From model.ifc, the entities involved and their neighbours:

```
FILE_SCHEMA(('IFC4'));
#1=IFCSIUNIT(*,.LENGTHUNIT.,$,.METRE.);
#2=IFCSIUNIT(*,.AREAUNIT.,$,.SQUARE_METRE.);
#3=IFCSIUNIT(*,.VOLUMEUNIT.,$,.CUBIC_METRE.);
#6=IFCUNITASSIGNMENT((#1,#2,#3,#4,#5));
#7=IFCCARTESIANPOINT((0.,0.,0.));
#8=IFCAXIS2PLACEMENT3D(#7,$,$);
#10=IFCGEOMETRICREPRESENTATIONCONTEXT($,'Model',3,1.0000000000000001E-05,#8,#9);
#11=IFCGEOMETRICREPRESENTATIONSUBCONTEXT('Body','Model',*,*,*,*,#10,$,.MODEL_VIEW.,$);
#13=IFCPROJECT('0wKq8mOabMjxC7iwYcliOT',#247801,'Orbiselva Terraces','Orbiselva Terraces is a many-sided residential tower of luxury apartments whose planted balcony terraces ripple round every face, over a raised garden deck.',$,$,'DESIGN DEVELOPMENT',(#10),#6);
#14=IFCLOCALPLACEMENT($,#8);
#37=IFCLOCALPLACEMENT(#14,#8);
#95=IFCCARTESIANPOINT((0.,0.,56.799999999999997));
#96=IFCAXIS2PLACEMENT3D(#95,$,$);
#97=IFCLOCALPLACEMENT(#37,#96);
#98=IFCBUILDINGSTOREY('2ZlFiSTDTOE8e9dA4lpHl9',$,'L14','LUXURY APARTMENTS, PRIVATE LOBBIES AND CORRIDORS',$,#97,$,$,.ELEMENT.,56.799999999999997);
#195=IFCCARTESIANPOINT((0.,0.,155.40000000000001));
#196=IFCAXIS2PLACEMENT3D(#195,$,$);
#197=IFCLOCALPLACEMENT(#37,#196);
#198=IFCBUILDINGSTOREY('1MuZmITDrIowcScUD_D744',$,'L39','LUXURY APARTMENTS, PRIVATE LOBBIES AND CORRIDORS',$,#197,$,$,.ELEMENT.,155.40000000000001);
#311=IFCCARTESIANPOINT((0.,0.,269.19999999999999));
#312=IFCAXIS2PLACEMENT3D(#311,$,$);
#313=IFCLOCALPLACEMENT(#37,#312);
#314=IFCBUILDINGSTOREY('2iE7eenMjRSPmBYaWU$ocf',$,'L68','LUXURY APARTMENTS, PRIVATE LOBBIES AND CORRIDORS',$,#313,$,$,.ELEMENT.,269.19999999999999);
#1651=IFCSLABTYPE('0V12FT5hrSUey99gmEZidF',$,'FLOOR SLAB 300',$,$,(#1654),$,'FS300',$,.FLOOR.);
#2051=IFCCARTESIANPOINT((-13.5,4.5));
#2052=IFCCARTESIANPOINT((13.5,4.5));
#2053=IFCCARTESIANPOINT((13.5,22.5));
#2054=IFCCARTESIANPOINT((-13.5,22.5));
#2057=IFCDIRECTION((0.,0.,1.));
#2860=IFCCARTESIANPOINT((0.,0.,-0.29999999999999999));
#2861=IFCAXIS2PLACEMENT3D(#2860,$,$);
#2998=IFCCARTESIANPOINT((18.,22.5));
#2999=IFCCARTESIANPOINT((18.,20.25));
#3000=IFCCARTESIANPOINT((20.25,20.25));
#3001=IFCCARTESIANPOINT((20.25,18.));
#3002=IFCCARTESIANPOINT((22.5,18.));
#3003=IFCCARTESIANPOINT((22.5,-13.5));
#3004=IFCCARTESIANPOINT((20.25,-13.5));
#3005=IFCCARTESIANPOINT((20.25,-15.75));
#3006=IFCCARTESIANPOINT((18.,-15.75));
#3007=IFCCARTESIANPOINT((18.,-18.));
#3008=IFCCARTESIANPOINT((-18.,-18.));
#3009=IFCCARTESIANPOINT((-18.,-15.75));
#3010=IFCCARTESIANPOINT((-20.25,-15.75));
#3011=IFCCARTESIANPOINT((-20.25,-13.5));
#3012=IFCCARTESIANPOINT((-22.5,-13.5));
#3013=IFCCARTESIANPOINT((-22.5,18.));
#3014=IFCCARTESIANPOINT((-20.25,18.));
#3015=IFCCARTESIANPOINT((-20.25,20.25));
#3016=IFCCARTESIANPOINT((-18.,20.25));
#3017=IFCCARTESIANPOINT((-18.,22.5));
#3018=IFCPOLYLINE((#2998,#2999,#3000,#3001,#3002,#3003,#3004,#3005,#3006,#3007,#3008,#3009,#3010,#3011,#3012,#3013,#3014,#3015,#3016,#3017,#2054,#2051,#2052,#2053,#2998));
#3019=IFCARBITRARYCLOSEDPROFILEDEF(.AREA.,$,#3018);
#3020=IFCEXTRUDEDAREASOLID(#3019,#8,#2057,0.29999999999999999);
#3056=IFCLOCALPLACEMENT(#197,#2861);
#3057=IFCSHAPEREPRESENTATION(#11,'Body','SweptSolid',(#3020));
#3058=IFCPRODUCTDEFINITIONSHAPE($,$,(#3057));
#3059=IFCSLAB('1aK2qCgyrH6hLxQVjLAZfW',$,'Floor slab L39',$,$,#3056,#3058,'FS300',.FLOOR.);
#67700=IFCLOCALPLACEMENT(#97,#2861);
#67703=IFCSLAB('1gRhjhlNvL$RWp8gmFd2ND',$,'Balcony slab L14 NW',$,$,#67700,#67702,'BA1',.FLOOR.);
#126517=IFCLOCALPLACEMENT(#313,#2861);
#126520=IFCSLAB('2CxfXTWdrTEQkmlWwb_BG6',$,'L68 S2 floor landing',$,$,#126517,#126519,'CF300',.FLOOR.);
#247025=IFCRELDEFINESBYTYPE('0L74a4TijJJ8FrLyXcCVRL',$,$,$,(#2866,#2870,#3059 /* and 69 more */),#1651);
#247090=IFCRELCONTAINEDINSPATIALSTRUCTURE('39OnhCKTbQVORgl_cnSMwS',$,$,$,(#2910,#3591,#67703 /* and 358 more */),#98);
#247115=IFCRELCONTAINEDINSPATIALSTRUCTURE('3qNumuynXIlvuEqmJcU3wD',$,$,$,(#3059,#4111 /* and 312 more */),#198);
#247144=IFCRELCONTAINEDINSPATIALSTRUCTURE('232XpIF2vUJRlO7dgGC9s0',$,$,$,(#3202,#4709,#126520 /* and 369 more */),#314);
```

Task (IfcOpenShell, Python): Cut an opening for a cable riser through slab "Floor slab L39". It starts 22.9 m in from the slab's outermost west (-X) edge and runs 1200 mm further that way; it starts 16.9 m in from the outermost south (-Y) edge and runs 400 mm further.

```python
import numpy as np
import ifcopenshell
import ifcopenshell.api.feature
import ifcopenshell.api.geometry
import ifcopenshell.api.root
import ifcopenshell.geom
import ifcopenshell.util.placement
import ifcopenshell.util.representation
import ifcopenshell.util.shape
import ifcopenshell.util.unit

model = ifcopenshell.open("model.ifc")
unit_scale = ifcopenshell.util.unit.calculate_unit_scale(model)
settings = ifcopenshell.geom.settings()


def volume(element):
    """Net volume in cubic metres, openings subtracted."""
    shape = ifcopenshell.geom.create_shape(settings, element)
    return ifcopenshell.util.shape.get_volume(shape.geometry)


slab = model.by_guid("1aK2qCgyrH6hLxQVjLAZfW")
before = volume(slab)

# Extent in the slab's own axes, in metres. The edges named are its -X and -Y sides.
slab_shape = ifcopenshell.geom.create_shape(settings, slab)
vertices = ifcopenshell.util.shape.get_vertices(slab_shape.geometry)
x_min, y_min, bottom = vertices.min(axis=0)
top = vertices[:, 2].max()

opening = ifcopenshell.api.root.create_entity(model, ifc_class="IfcOpeningElement", name="Cable riser opening", predefined_type="OPENING")
context = ifcopenshell.util.representation.get_context(model, "Model", "Body", "MODEL_VIEW")
width, depth = 1.2, 0.4
outline = [(0.0, 0.0), (width, 0.0), (width, depth), (0.0, depth), (0.0, 0.0)]
# Overshoot both faces by 50 mm so the cut is clean.
shape = ifcopenshell.api.geometry.add_slab_representation(
    model, context=context, depth=top - bottom + 0.1, polyline=outline
)
ifcopenshell.api.geometry.assign_representation(model, product=opening, representation=shape)

matrix = ifcopenshell.util.placement.get_local_placement(slab.ObjectPlacement)
matrix[:, 3] = matrix @ np.append(np.array([x_min + 22.9, y_min + 16.9, bottom - 0.05]) / unit_scale, 1.0)
ifcopenshell.api.geometry.edit_object_placement(model, product=opening, matrix=matrix, is_si=False)
ifcopenshell.api.feature.add_feature(model, feature=opening, element=slab)

after = volume(slab)

print(f"slab volume {before:.3f} -> {after:.3f} m3")

model.write("model-out.ifc")
```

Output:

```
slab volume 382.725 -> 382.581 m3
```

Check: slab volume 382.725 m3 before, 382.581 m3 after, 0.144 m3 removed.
